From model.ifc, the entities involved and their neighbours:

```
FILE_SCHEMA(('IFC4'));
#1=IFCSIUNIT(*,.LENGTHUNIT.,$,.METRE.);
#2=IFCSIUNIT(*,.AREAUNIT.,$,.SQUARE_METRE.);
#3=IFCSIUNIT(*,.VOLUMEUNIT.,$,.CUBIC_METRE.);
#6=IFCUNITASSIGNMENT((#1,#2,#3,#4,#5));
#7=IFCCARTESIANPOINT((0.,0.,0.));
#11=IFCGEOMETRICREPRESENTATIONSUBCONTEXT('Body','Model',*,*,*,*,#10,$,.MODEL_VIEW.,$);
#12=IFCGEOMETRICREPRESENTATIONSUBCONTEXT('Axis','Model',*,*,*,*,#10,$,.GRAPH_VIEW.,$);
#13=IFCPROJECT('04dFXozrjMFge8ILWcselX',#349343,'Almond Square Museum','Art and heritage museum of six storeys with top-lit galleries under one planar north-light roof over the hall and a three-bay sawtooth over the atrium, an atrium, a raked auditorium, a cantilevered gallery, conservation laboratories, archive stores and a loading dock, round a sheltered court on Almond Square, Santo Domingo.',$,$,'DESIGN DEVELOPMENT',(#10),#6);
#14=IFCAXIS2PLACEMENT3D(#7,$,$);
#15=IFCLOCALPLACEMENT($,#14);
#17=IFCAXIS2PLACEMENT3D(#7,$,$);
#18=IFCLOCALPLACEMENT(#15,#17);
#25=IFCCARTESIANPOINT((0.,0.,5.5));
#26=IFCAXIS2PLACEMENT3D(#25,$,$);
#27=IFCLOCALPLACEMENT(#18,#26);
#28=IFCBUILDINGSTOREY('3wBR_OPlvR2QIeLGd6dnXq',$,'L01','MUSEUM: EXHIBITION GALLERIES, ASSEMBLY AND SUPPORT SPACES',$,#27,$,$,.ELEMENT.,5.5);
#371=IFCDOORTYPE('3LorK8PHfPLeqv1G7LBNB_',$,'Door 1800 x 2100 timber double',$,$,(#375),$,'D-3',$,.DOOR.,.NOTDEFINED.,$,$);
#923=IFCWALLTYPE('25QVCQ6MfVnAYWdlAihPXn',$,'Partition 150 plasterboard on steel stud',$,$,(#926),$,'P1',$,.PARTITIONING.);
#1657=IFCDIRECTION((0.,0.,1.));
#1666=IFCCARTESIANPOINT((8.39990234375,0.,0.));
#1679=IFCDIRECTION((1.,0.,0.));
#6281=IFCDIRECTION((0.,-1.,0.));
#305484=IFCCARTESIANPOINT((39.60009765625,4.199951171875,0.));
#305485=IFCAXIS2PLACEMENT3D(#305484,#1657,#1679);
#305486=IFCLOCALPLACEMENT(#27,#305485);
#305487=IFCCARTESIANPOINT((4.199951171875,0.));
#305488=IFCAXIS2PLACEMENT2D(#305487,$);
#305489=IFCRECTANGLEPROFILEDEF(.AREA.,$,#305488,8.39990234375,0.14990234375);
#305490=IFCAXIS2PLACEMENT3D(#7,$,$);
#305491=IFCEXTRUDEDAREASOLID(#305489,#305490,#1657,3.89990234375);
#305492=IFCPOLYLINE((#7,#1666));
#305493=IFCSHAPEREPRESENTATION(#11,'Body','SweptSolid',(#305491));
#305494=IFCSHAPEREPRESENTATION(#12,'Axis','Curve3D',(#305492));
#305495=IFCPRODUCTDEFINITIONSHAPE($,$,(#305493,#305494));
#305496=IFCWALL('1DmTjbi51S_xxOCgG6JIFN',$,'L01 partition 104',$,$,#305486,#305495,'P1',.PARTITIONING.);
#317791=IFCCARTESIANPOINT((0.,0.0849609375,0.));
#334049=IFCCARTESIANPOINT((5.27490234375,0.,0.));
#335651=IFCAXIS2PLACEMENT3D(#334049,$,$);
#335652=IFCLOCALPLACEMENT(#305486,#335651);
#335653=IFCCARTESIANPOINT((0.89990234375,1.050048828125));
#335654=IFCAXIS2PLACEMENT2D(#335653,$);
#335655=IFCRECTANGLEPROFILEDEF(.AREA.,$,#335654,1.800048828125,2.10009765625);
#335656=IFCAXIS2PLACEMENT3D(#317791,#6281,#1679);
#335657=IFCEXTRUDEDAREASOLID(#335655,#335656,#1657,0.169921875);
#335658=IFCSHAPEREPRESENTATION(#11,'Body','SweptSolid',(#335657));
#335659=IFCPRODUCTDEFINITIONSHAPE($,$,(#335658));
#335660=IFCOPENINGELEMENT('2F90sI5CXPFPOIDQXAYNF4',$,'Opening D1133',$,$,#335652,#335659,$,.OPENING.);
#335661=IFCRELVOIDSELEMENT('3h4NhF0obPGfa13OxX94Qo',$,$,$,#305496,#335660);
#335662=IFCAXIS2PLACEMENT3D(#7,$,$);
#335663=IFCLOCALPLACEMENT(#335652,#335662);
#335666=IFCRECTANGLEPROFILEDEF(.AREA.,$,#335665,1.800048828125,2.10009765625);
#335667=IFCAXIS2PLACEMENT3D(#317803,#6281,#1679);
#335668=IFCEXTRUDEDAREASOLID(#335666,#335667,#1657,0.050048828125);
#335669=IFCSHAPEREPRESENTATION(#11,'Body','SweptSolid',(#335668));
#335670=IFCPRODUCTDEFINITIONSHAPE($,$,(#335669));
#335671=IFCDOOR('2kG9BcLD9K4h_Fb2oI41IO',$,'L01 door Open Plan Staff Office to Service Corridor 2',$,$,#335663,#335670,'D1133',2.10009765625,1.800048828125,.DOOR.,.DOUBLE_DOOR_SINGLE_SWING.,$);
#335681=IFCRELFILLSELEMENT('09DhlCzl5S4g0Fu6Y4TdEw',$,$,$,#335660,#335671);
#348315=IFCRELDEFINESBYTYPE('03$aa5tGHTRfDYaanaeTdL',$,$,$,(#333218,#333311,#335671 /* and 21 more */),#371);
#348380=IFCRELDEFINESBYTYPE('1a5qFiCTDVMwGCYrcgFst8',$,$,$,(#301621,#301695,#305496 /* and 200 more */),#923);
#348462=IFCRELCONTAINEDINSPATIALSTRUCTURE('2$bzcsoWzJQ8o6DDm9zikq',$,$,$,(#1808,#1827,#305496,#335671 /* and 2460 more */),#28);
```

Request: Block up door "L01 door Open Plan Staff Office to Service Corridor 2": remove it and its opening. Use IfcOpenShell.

```python
import ifcopenshell
import ifcopenshell.api.feature
import ifcopenshell.api.root
import ifcopenshell.geom
import ifcopenshell.util.shape

model = ifcopenshell.open("model.ifc")
settings = ifcopenshell.geom.settings()


def volume(element):
    """Net volume in cubic metres, openings subtracted."""
    shape = ifcopenshell.geom.create_shape(settings, element)
    return ifcopenshell.util.shape.get_volume(shape.geometry)


door = model.by_guid("2kG9BcLD9K4h_Fb2oI41IO")
opening = door.FillsVoids[0].RelatingOpeningElement
wall = opening.VoidsElements[0].RelatingBuildingElement
before = volume(wall)

ifcopenshell.api.root.remove_product(model, product=door)
ifcopenshell.api.feature.remove_feature(model, feature=opening)

after = volume(wall)

print(f"wall volume {before:.3f} -> {after:.3f} m3")

model.write("model_updated.ifc")
```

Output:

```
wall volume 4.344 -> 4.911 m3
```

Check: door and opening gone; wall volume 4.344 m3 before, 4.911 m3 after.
